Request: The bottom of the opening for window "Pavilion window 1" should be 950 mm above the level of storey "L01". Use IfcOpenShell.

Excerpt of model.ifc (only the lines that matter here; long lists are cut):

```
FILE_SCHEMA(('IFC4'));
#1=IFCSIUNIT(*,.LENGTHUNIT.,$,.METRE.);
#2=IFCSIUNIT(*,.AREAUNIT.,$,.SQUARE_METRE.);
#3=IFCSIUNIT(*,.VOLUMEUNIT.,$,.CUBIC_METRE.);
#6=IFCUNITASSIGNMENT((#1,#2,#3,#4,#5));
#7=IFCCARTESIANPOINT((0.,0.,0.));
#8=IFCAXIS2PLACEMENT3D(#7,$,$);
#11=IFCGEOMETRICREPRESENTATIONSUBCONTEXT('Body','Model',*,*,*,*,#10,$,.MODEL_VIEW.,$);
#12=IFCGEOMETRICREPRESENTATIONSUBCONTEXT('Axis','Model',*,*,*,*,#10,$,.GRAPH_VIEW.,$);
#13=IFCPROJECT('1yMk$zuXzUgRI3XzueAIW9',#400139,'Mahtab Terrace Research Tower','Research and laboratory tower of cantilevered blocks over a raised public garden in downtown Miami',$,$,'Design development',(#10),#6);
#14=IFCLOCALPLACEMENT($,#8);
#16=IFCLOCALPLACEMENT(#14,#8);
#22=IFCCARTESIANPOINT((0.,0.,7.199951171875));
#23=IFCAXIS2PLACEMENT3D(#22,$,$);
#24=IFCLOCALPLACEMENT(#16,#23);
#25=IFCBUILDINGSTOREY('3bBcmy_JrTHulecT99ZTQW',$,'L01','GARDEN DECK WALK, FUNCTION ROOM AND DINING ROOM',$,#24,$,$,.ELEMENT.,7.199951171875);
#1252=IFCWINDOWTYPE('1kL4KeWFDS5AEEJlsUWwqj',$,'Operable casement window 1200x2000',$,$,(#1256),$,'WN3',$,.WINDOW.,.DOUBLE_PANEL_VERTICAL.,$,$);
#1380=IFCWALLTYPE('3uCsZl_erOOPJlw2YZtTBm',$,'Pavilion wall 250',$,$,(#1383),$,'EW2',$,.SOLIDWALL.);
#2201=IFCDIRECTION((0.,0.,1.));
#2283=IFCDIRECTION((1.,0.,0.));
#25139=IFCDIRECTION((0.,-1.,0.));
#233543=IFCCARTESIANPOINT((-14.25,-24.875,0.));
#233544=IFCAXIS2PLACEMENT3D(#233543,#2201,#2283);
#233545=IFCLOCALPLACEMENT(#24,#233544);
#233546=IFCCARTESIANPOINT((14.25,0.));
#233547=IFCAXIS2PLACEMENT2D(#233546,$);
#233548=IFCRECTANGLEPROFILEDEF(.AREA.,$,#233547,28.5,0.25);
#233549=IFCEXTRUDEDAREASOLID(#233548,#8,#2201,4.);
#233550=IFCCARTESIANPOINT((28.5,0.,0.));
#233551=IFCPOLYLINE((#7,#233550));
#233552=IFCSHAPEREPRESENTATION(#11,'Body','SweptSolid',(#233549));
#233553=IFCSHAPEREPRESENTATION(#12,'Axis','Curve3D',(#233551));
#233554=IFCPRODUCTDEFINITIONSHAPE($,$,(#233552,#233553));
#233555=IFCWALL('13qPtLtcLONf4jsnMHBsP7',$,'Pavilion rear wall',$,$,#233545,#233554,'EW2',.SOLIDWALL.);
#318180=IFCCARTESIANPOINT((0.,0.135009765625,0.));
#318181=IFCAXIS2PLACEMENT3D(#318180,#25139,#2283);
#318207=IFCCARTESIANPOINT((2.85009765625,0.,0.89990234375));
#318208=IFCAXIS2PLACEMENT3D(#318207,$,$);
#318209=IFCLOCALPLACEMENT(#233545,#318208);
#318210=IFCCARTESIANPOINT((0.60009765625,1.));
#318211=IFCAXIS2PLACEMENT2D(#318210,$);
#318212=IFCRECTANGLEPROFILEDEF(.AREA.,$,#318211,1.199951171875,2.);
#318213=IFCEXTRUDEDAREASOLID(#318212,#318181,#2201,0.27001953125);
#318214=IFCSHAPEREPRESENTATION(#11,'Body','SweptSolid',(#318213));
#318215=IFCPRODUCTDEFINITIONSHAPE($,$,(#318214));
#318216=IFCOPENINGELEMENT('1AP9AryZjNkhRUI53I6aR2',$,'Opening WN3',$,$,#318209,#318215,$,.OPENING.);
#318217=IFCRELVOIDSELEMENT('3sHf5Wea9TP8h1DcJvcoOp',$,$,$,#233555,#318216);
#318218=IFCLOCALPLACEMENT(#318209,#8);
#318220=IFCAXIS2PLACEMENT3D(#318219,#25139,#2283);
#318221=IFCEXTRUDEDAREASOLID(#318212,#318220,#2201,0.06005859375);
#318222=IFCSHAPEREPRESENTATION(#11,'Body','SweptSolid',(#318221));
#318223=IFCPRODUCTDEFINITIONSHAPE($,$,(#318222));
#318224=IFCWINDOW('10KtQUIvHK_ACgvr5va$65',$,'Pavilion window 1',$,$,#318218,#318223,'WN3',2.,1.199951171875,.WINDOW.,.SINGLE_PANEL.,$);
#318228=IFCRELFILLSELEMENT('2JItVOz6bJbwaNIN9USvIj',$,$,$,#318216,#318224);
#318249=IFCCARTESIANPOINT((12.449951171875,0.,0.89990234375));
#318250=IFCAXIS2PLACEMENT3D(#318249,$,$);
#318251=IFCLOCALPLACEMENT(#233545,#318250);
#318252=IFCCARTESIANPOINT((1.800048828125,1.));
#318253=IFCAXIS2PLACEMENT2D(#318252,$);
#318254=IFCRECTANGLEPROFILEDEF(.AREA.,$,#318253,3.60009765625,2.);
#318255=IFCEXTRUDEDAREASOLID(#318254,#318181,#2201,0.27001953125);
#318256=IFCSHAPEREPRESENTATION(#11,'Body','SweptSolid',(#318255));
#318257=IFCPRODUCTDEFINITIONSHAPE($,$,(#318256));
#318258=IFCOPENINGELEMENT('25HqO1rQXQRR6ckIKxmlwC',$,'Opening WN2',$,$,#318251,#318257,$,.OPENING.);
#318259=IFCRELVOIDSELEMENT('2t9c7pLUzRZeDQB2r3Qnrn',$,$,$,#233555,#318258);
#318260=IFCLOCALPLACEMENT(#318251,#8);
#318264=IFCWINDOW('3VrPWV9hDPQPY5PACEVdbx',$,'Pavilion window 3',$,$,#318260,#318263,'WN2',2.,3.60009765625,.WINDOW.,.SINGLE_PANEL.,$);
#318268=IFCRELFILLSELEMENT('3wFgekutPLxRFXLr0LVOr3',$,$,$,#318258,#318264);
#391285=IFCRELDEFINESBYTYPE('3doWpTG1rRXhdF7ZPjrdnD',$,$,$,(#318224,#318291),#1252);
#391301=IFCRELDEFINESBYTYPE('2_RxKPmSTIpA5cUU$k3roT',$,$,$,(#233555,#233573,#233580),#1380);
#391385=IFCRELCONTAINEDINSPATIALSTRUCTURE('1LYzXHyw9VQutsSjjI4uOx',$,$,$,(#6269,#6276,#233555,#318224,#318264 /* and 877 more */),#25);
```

```python
import numpy as np
import ifcopenshell
import ifcopenshell.api.geometry
import ifcopenshell.geom
import ifcopenshell.util.element
import ifcopenshell.util.placement
import ifcopenshell.util.shape
import ifcopenshell.util.unit

model = ifcopenshell.open("model.ifc")
unit_scale = ifcopenshell.util.unit.calculate_unit_scale(model)

window = model.by_guid("10KtQUIvHK_ACgvr5va$65")
opening = window.FillsVoids[0].RelatingOpeningElement
storey = ifcopenshell.util.element.get_container(window, ifc_class="IfcBuildingStorey")
level = ifcopenshell.util.placement.get_local_placement(storey.ObjectPlacement)[2, 3]

# The opening's origin need not be at the sill, so measure its lowest point.
shape = ifcopenshell.geom.create_shape(ifcopenshell.geom.settings(), opening)
bottom = ifcopenshell.util.shape.get_shape_bottom_elevation(shape, shape.geometry) / unit_scale
dz = level + 0.95 - bottom

shift = np.array([0.0, 0.0, dz])
# The window is placed relative to its opening, so it follows when the opening moves.
matrix = ifcopenshell.util.placement.get_local_placement(opening.ObjectPlacement)
matrix[:3, 3] += shift
ifcopenshell.api.geometry.edit_object_placement(
    model, product=opening, matrix=matrix, is_si=False, should_transform_children=True
)

print(f"moved by {dz * unit_scale:+.3f} m")

model.write("model_rev.ifc")
```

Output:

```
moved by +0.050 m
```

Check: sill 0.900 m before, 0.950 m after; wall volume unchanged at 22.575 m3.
